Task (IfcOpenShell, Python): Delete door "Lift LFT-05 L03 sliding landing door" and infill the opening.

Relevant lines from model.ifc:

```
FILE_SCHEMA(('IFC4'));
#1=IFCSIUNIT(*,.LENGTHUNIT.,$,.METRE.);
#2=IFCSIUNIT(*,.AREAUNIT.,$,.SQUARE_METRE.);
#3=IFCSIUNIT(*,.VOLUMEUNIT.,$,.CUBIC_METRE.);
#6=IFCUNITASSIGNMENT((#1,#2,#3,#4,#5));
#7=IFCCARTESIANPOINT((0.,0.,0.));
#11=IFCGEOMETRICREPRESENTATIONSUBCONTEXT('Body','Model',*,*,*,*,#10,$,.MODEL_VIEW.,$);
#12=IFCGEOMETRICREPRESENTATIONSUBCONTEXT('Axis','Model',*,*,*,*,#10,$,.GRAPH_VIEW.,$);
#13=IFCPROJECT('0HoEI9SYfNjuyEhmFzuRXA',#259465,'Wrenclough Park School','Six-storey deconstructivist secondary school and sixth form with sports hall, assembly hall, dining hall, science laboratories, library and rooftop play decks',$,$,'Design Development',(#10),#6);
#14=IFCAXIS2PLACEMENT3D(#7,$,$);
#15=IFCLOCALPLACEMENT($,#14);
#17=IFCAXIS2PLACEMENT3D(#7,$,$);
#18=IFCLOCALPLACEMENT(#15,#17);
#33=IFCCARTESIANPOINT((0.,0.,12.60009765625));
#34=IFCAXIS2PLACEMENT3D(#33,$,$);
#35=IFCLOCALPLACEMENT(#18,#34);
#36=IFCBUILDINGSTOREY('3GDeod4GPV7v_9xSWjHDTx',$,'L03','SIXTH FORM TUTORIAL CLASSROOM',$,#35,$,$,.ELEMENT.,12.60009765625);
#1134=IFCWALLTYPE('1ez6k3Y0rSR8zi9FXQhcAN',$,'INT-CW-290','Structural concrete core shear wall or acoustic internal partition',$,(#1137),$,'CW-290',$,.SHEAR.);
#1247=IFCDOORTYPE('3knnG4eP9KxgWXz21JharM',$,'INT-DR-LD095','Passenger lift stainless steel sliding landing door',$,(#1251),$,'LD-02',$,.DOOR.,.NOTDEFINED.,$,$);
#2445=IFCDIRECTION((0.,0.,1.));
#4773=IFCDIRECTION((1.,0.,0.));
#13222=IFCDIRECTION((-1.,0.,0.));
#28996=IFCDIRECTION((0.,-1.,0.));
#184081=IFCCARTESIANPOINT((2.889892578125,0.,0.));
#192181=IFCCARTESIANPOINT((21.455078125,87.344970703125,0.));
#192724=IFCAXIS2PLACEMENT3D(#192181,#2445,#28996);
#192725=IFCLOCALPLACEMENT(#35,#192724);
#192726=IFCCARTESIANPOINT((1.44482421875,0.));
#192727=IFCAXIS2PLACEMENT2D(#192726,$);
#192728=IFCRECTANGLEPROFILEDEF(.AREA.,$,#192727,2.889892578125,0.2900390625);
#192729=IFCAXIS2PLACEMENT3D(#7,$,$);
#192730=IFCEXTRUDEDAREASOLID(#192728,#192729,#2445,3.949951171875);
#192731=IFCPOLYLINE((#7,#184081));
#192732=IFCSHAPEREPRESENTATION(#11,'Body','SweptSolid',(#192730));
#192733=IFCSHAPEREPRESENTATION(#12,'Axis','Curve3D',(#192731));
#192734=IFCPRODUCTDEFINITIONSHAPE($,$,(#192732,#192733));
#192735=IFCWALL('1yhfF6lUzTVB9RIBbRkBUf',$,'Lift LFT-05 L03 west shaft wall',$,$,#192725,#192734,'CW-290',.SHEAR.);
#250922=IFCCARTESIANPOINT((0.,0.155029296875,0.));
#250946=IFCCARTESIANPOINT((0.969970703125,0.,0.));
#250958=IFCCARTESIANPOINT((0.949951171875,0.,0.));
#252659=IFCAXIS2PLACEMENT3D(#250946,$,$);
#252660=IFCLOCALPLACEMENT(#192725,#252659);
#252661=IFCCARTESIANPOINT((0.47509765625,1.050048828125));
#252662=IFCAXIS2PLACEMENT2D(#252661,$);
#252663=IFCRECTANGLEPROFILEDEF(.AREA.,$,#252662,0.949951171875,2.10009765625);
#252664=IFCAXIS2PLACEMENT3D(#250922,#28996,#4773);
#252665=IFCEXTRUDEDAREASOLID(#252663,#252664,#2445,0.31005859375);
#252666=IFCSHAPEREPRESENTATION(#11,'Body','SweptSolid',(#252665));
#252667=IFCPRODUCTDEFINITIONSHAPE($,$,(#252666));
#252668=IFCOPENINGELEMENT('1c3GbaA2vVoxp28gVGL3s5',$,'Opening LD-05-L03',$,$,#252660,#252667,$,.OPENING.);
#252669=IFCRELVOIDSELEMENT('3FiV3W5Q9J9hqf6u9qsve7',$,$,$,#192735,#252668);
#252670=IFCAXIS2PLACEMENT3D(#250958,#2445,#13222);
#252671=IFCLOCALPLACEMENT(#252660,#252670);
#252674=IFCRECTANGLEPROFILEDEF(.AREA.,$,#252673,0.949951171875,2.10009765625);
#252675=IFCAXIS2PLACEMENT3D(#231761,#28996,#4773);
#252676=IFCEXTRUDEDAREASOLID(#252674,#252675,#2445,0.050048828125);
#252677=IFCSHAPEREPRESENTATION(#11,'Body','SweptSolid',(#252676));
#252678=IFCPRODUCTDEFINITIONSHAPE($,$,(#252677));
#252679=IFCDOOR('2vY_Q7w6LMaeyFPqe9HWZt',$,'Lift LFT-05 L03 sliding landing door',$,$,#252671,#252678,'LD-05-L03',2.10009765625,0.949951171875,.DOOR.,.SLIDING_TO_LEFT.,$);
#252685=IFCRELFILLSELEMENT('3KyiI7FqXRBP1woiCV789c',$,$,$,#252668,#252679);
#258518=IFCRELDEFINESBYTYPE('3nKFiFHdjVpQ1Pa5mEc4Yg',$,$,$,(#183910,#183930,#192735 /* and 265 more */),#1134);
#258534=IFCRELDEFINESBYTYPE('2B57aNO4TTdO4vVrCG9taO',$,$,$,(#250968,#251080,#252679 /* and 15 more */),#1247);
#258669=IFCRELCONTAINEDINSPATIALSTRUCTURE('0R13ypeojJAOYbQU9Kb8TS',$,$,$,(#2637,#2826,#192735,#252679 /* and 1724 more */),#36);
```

```python
import ifcopenshell
import ifcopenshell.api.feature
import ifcopenshell.api.root
import ifcopenshell.geom
import ifcopenshell.util.shape

model = ifcopenshell.open("model.ifc")
settings = ifcopenshell.geom.settings()


def volume(element):
    """Net volume in cubic metres, openings subtracted."""
    shape = ifcopenshell.geom.create_shape(settings, element)
    return ifcopenshell.util.shape.get_volume(shape.geometry)


door = model.by_guid("2vY_Q7w6LMaeyFPqe9HWZt")
opening = door.FillsVoids[0].RelatingOpeningElement
wall = opening.VoidsElements[0].RelatingBuildingElement
before = volume(wall)

ifcopenshell.api.root.remove_product(model, product=door)
ifcopenshell.api.feature.remove_feature(model, feature=opening)

after = volume(wall)

print(f"wall volume {before:.3f} -> {after:.3f} m3")

model.write("model-out.ifc")
```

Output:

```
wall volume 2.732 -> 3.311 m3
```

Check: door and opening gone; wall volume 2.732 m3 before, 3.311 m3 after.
